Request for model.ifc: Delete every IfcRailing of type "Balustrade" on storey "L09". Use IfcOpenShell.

First a look at what the model holds.

```python
import ifcopenshell
import ifcopenshell.util.element

model = ifcopenshell.open("model.ifc")
print(model.schema)
storey = next(s for s in model.by_type("IfcBuildingStorey") if s.Name == "L09")
railings = [e for e in ifcopenshell.util.element.get_decomposition(storey) if e.is_a("IfcRailing")]
seen = {}
for e in railings:
    element_type = ifcopenshell.util.element.get_type(e)
    name = element_type.Name if element_type not in (None, e) else None
    seen[name] = seen.get(name, 0) + 1
for name, count in sorted(seen.items(), key=str):
    print(count, "x", name)
```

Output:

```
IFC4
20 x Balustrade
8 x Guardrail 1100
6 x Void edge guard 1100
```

```python
import ifcopenshell
import ifcopenshell.api.root
import ifcopenshell.util.element

model = ifcopenshell.open("model.ifc")

storey = next(s for s in model.by_type("IfcBuildingStorey") if s.Name == "L09")
railings = [e for e in ifcopenshell.util.element.get_decomposition(storey) if e.is_a("IfcRailing")]
targets = [e for e in railings if (t := ifcopenshell.util.element.get_type(e)) not in (None, e) and t.Name == "Balustrade"]

for e in targets:
    ifcopenshell.api.root.remove_product(model, product=e)
print(len(targets), "removed")

model.write("model_v2.ifc")
```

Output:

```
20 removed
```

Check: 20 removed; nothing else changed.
